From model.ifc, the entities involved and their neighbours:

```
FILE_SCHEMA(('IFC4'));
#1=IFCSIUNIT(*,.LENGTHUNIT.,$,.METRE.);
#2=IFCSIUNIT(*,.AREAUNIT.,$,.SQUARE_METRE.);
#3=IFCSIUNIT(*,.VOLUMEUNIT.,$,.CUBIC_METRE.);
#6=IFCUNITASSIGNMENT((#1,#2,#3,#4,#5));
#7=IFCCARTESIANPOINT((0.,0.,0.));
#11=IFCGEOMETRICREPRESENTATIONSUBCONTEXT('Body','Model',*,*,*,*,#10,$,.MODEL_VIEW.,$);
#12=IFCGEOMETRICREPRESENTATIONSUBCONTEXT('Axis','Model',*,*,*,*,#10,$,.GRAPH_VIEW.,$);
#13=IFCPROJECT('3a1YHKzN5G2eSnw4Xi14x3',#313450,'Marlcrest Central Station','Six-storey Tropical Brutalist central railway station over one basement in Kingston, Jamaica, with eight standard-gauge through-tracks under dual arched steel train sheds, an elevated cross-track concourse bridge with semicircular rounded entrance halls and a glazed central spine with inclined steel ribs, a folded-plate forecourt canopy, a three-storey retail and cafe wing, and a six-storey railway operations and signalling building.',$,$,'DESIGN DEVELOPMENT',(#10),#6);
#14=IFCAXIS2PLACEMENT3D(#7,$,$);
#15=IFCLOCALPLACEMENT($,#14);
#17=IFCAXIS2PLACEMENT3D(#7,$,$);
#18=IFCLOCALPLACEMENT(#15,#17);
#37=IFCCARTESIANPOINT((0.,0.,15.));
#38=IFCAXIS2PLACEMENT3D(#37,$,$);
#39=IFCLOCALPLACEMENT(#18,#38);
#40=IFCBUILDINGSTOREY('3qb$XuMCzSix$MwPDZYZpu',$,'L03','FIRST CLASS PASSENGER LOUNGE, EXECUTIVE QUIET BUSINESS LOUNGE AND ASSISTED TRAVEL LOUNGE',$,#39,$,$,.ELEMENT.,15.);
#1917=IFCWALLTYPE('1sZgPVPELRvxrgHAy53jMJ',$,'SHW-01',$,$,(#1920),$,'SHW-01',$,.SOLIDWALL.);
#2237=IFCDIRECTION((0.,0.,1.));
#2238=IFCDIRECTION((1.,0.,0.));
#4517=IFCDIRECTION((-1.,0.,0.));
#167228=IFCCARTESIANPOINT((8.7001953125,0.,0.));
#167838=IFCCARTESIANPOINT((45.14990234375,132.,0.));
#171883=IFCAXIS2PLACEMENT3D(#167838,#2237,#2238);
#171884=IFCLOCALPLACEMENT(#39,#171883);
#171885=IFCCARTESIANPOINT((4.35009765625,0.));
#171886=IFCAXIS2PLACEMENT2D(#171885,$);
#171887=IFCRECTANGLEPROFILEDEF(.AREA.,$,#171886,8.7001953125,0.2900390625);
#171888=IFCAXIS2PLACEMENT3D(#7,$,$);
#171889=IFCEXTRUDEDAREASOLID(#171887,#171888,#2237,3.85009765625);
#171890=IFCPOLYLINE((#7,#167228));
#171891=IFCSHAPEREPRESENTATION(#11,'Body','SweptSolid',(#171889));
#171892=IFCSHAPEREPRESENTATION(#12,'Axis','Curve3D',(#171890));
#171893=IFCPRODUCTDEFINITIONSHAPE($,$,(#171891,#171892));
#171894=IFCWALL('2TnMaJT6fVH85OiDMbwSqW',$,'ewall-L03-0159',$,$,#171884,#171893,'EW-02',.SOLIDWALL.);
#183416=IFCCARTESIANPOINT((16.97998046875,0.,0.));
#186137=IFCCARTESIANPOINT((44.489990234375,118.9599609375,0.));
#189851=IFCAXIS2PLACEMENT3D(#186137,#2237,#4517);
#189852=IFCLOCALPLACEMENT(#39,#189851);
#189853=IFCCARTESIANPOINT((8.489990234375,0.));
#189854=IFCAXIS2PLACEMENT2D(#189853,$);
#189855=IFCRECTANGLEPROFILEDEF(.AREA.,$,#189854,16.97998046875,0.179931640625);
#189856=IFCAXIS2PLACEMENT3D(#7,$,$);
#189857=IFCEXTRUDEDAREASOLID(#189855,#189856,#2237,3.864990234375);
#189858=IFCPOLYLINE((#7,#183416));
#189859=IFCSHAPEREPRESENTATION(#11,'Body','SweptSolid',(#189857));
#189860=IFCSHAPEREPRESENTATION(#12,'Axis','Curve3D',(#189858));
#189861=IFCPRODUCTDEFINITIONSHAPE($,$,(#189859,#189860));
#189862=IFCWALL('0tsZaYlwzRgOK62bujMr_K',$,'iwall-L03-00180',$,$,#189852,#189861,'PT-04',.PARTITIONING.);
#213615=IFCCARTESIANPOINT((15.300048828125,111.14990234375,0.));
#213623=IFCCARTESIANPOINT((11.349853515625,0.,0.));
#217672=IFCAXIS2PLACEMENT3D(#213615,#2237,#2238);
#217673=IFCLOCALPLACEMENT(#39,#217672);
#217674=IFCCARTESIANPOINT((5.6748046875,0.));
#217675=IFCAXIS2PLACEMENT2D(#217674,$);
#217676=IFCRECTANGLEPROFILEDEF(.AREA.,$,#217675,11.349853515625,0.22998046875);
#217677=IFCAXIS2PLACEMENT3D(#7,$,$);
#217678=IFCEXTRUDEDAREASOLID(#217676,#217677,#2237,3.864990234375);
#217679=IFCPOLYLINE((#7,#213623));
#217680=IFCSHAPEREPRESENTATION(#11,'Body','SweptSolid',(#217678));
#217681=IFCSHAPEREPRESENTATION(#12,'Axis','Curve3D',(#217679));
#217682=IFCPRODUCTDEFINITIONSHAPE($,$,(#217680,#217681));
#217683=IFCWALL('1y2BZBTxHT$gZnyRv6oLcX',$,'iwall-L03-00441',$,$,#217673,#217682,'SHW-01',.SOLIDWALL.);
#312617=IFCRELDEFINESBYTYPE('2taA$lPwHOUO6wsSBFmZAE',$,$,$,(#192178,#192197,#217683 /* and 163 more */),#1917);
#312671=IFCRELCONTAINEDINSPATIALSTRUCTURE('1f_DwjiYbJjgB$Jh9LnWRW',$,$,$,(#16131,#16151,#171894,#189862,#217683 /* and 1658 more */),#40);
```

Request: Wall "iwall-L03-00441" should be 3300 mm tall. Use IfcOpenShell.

```python
import ifcopenshell
import ifcopenshell.geom
import ifcopenshell.util.representation
import ifcopenshell.util.shape

model = ifcopenshell.open("model.ifc")
settings = ifcopenshell.geom.settings()


def volume(element):
    """Net volume in cubic metres, openings subtracted."""
    shape = ifcopenshell.geom.create_shape(settings, element)
    return ifcopenshell.util.shape.get_volume(shape.geometry)


wall = model.by_id(217683)
before = volume(wall)

body = ifcopenshell.util.representation.get_representation(wall, "Model", "Body")
solid = body.Items[0]
old_height = solid.Depth
solid.Depth = 3.3
after = volume(wall)

print(f"height {old_height:g} -> {solid.Depth:g}, volume {before:.3f} -> {after:.3f} m3")

model.write("model_updated.ifc")
```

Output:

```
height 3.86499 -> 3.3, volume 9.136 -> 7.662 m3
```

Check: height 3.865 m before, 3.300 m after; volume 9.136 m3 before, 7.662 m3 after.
